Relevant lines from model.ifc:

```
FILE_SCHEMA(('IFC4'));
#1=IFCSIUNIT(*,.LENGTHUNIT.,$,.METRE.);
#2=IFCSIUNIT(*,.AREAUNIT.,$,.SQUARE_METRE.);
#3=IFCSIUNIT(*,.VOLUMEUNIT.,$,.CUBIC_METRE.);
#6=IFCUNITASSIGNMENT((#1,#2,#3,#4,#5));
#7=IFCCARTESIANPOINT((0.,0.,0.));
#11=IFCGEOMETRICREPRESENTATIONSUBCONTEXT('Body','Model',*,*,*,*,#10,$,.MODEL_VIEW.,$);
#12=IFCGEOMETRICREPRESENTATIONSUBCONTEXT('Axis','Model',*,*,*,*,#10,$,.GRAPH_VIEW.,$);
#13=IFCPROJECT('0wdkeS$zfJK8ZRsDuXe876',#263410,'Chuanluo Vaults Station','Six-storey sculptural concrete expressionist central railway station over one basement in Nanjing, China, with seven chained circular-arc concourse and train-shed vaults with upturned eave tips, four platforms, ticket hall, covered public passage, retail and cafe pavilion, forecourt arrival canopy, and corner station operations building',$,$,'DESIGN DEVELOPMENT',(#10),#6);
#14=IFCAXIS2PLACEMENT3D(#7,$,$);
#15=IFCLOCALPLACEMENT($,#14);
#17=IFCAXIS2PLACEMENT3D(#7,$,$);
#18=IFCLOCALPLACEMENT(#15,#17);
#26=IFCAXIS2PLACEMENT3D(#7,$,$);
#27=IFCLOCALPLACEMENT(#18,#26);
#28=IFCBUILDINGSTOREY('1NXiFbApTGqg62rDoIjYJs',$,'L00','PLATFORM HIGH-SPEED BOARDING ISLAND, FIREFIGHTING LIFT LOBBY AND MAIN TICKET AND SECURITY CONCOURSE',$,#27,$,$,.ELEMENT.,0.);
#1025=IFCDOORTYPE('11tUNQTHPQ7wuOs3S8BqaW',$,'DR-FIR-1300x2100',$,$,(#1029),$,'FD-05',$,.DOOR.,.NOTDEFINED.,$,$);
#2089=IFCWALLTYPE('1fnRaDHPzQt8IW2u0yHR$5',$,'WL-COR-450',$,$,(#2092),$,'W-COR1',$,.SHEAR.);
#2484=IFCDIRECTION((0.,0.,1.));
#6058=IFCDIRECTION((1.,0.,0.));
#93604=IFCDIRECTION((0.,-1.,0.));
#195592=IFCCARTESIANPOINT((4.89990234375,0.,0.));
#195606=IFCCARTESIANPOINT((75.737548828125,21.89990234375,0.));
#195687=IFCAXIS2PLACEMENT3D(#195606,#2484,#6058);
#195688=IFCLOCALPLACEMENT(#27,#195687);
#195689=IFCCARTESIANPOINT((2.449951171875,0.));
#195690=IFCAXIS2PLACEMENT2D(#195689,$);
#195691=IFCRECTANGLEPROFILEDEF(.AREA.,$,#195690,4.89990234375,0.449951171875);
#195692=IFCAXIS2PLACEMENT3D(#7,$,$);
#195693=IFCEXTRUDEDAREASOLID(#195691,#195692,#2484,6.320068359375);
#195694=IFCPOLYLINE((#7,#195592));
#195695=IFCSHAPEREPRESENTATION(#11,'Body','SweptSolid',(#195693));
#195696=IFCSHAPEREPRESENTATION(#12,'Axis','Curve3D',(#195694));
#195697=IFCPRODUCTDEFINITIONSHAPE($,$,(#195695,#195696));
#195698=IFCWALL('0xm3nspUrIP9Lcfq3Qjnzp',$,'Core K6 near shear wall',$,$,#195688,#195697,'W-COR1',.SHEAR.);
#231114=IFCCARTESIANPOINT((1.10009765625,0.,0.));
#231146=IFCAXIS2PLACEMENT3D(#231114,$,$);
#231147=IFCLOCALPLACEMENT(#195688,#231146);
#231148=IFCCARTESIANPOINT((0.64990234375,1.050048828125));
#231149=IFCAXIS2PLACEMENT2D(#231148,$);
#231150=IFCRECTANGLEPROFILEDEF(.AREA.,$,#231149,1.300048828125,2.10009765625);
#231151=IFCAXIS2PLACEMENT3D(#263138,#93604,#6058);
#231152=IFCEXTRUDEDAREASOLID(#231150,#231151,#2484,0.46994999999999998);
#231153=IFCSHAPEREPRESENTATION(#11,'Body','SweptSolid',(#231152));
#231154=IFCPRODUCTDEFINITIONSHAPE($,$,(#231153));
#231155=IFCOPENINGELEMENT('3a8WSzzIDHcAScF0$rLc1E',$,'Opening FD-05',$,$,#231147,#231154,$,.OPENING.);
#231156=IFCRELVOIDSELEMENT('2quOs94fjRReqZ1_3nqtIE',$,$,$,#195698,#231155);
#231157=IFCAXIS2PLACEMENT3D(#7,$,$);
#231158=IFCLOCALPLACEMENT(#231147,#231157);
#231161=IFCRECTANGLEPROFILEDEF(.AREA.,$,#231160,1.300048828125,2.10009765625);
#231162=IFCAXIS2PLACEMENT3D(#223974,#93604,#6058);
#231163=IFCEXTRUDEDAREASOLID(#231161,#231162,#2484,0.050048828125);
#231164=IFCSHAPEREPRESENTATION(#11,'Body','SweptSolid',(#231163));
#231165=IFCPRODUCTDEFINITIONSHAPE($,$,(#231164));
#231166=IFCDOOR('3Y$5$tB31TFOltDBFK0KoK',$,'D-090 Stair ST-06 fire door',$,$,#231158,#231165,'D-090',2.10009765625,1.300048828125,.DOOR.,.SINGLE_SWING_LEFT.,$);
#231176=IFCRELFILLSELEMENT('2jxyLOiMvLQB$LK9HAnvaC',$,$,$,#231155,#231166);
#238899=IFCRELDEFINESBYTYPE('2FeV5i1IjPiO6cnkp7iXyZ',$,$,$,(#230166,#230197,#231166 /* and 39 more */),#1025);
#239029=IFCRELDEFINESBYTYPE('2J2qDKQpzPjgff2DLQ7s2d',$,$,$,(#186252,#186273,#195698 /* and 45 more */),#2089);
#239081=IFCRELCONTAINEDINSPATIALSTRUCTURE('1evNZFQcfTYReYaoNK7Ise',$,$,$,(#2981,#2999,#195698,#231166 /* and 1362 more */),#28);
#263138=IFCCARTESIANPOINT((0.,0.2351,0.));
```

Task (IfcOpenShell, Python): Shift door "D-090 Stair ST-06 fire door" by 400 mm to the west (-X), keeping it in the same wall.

```python
import ifcopenshell
import ifcopenshell.api.geometry
import ifcopenshell.util.placement
import ifcopenshell.util.unit

model = ifcopenshell.open("model.ifc")
unit_scale = ifcopenshell.util.unit.calculate_unit_scale(model)

door = model.by_guid("3Y$5$tB31TFOltDBFK0KoK")
opening = door.FillsVoids[0].RelatingOpeningElement
wall = opening.VoidsElements[0].RelatingBuildingElement

wall_matrix = ifcopenshell.util.placement.get_local_placement(wall.ObjectPlacement)
shift = wall_matrix[:3, 0] * -0.4 / unit_scale
before = ifcopenshell.util.placement.get_local_placement(door.ObjectPlacement)[:3, 3].copy()

# The door is placed relative to its opening, so it follows when the opening moves.
matrix = ifcopenshell.util.placement.get_local_placement(opening.ObjectPlacement)
matrix[:3, 3] += shift
ifcopenshell.api.geometry.edit_object_placement(
    model, product=opening, matrix=matrix, is_si=False, should_transform_children=True
)

after = ifcopenshell.util.placement.get_local_placement(door.ObjectPlacement)[:3, 3]
print("door moved by", (after - before).round(3) + 0.0)

model.write("model_updated.ifc")
```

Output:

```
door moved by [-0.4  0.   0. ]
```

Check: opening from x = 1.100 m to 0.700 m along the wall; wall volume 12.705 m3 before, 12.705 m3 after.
